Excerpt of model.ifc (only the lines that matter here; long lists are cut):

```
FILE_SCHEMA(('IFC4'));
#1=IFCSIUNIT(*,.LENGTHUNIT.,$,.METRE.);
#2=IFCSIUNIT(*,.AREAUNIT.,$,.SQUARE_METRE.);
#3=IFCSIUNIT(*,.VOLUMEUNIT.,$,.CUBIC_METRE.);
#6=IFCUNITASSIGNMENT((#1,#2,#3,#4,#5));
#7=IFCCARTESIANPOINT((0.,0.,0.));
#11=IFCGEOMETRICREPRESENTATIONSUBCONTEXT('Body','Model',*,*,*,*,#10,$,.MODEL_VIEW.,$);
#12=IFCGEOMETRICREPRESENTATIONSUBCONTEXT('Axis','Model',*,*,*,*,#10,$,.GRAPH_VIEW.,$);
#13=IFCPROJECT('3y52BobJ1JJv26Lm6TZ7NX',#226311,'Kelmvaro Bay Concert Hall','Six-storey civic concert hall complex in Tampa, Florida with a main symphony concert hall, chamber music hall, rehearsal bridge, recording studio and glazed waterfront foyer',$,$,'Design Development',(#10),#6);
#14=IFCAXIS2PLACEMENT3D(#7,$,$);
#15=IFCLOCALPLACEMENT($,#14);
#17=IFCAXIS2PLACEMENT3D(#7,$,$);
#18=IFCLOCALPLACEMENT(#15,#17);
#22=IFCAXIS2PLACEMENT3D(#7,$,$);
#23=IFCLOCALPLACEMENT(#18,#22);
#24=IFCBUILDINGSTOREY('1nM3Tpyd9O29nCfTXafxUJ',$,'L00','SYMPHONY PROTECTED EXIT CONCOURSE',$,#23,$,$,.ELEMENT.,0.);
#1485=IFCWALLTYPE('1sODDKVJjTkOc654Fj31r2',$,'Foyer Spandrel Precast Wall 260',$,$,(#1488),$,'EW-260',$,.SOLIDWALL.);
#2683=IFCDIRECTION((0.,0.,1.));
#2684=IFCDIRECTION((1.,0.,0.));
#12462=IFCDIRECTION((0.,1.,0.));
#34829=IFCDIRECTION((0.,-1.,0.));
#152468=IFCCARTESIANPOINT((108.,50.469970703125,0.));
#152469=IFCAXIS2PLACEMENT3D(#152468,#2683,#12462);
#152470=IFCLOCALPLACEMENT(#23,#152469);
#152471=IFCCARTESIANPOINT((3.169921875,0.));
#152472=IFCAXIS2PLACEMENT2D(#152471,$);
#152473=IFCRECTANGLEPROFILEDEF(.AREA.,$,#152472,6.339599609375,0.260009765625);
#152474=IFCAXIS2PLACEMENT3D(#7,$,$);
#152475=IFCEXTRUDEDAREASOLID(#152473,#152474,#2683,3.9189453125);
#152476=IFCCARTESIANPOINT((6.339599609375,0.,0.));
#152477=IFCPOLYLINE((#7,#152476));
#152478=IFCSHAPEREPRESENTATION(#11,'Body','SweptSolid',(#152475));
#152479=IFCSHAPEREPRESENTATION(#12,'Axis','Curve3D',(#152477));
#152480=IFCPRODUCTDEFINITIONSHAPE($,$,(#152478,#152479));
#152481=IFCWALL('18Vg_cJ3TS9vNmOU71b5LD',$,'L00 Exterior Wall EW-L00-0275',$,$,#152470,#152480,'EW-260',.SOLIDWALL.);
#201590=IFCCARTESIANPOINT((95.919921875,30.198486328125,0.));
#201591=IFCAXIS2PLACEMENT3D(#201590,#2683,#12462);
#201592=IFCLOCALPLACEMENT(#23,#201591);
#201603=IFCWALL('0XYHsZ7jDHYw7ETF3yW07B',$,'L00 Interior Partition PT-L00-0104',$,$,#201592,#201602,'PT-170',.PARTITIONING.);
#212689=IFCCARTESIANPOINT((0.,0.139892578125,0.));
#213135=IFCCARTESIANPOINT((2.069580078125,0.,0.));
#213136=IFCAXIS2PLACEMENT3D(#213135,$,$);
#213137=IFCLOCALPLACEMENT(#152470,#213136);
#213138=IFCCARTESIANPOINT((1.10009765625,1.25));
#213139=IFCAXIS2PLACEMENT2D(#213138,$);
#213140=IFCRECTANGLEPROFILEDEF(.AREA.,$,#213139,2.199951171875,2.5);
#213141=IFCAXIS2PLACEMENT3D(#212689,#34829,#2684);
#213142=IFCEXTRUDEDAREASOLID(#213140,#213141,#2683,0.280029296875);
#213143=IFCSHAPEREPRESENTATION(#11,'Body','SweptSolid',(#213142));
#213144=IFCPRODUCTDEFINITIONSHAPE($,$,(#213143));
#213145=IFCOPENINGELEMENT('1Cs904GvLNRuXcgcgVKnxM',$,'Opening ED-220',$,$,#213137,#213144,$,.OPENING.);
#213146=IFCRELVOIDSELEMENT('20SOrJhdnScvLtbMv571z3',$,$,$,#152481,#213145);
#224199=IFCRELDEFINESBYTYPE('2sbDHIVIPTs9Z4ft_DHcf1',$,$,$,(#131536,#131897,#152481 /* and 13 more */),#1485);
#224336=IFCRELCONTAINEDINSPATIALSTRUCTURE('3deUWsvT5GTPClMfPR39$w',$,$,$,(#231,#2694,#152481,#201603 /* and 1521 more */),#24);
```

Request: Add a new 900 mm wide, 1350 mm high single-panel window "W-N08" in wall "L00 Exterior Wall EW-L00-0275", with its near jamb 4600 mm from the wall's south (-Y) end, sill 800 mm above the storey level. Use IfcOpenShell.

```python
import numpy as np
import ifcopenshell
import ifcopenshell.api.feature
import ifcopenshell.api.geometry
import ifcopenshell.api.root
import ifcopenshell.api.spatial
import ifcopenshell.geom
import ifcopenshell.util.element
import ifcopenshell.util.placement
import ifcopenshell.util.representation
import ifcopenshell.util.shape
import ifcopenshell.util.unit

model = ifcopenshell.open("model.ifc")
unit_scale = ifcopenshell.util.unit.calculate_unit_scale(model)
settings = ifcopenshell.geom.settings()


def volume(element):
    """Net volume in cubic metres, openings subtracted."""
    shape = ifcopenshell.geom.create_shape(settings, element)
    return ifcopenshell.util.shape.get_volume(shape.geometry)


wall = model.by_guid("18Vg_cJ3TS9vNmOU71b5LD")
storey = ifcopenshell.util.element.get_container(wall, ifc_class="IfcBuildingStorey")
context = ifcopenshell.util.representation.get_context(model, "Model", "Body", "MODEL_VIEW")
before = volume(wall)

width, height, from_end, sill = 0.9, 1.35, 4.6, 0.8  # metres

# The wall runs along its own X axis, and the end named is its -X end.
wall_shape = ifcopenshell.geom.create_shape(settings, wall)
x, y, z = ifcopenshell.util.shape.get_vertices(wall_shape.geometry).T
start = x.min() + from_end
face, thickness = float(y.min()), float(y.max() - y.min())
wall_matrix = ifcopenshell.util.placement.get_local_placement(wall.ObjectPlacement)
level = ifcopenshell.util.placement.get_local_placement(storey.ObjectPlacement)[2, 3]


def in_wall(x, y):
    """Placement at x, y metres in the wall's axes, at sill height."""
    matrix = wall_matrix.copy()
    matrix[:, 3] = wall_matrix @ np.array([x / unit_scale, y / unit_scale, 0.0, 1.0])
    matrix[2, 3] = level + sill / unit_scale
    return matrix


# Opening: a box that overshoots both wall faces by 50 mm.
opening = ifcopenshell.api.root.create_entity(model, ifc_class="IfcOpeningElement", predefined_type="OPENING")
box = ifcopenshell.api.geometry.add_wall_representation(
    model, context=context, length=width, height=height, thickness=thickness + 0.1
)
ifcopenshell.api.geometry.assign_representation(model, product=opening, representation=box)
ifcopenshell.api.geometry.edit_object_placement(model, product=opening, matrix=in_wall(start, face - 0.05), is_si=False)
ifcopenshell.api.feature.add_feature(model, feature=opening, element=wall)

window = ifcopenshell.api.root.create_entity(model, ifc_class="IfcWindow", name="W-N08", predefined_type="WINDOW")
window.OverallWidth, window.OverallHeight = width / unit_scale, height / unit_scale
window.PartitioningType = "SINGLE_PANEL"
body = ifcopenshell.api.geometry.add_window_representation(
    model,
    context=context,
    overall_width=window.OverallWidth,
    overall_height=window.OverallHeight,
    partition_type="SINGLE_PANEL",
)
ifcopenshell.api.geometry.assign_representation(model, product=window, representation=body)
ifcopenshell.api.spatial.assign_container(model, products=[window], relating_structure=storey)
ifcopenshell.api.feature.add_filling(model, opening=opening, element=window)

# Centre the window in the wall's thickness.
ifcopenshell.api.geometry.edit_object_placement(model, product=window, matrix=in_wall(start, face), is_si=False)
window_shape = ifcopenshell.geom.create_shape(settings, window)
depth = ifcopenshell.util.shape.get_vertices(window_shape.geometry)[:, 1]
offset = face + thickness / 2 - (depth.min() + depth.max()) / 2
ifcopenshell.api.geometry.edit_object_placement(model, product=window, matrix=in_wall(start, offset), is_si=False)

after = volume(wall)

print(f"wall volume {before:.3f} -> {after:.3f} m3")

model.write("model_rev.ifc")
```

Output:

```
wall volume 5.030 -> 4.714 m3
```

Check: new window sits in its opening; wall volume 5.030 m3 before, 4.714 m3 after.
